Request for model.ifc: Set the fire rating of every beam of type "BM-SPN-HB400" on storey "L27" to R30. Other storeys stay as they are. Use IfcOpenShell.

First a look at what the model holds.

```python
import ifcopenshell
import ifcopenshell.util.element

model = ifcopenshell.open("model.ifc")
print(model.schema)
storey = next(s for s in model.by_type("IfcBuildingStorey") if s.Name == "L27")
beams = [e for e in ifcopenshell.util.element.get_decomposition(storey) if e.is_a("IfcBeam")]
seen = {}
for e in beams:
    element_type = ifcopenshell.util.element.get_type(e)
    key = (element_type.Name if element_type != e and element_type else None, ifcopenshell.util.element.get_pset(e, "Pset_BeamCommon", "FireRating"))
    seen[key] = seen.get(key, 0) + 1
for (name, value), count in sorted(seen.items(), key=str):
    print(count, "x", name, "|", value)
```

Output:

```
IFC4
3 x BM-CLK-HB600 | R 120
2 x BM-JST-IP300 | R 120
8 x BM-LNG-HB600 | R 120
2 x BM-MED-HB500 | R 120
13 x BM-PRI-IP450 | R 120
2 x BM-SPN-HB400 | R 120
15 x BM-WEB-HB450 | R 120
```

```python
import ifcopenshell
import ifcopenshell.api.pset
import ifcopenshell.util.element

model = ifcopenshell.open("model.ifc")

storey = next(s for s in model.by_type("IfcBuildingStorey") if s.Name == "L27")
beams = [e for e in ifcopenshell.util.element.get_decomposition(storey) if e.is_a("IfcBeam")]

count = 0
for e in beams:
    element_type = ifcopenshell.util.element.get_type(e)
    if element_type in (None, e) or element_type.Name != "BM-SPN-HB400":
        continue
    found = ifcopenshell.util.element.get_pset(e, "Pset_BeamCommon", should_inherit=False)
    if found:
        pset = model.by_id(found["id"])
        if len(ifcopenshell.util.element.get_elements_by_pset(pset)) > 1:
            pset = ifcopenshell.api.pset.unshare_pset(model, products=[e], pset=pset)[0]
    else:
        pset = ifcopenshell.api.pset.add_pset(model, product=e, name="Pset_BeamCommon")
    ifcopenshell.api.pset.edit_pset(model, pset=pset, properties={"FireRating": "R30"})
    count += 1

print(count, "beams updated")

model.write("model-out.ifc")
```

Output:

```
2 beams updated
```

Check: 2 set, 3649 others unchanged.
